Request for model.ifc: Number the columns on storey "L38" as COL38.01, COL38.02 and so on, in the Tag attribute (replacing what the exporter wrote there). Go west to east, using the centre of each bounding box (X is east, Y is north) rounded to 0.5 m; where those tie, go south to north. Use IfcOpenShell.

First a look at what the model holds.

```python
import ifcopenshell
import ifcopenshell.util.element
import ifcopenshell.util.placement

model = ifcopenshell.open("model.ifc")
print(model.schema)
storey = next(s for s in model.by_type("IfcBuildingStorey") if s.Name == "L38")
columns = [e for e in ifcopenshell.util.element.get_decomposition(storey) if e.is_a("IfcColumn")]
for e in sorted(columns, key=lambda e: e.id()):
    origin = ifcopenshell.util.placement.get_local_placement(e.ObjectPlacement)[:3, 3]
    print(e.id(), e.Tag, e.Name, origin.round(2) + 0.0, sep=" | ")
```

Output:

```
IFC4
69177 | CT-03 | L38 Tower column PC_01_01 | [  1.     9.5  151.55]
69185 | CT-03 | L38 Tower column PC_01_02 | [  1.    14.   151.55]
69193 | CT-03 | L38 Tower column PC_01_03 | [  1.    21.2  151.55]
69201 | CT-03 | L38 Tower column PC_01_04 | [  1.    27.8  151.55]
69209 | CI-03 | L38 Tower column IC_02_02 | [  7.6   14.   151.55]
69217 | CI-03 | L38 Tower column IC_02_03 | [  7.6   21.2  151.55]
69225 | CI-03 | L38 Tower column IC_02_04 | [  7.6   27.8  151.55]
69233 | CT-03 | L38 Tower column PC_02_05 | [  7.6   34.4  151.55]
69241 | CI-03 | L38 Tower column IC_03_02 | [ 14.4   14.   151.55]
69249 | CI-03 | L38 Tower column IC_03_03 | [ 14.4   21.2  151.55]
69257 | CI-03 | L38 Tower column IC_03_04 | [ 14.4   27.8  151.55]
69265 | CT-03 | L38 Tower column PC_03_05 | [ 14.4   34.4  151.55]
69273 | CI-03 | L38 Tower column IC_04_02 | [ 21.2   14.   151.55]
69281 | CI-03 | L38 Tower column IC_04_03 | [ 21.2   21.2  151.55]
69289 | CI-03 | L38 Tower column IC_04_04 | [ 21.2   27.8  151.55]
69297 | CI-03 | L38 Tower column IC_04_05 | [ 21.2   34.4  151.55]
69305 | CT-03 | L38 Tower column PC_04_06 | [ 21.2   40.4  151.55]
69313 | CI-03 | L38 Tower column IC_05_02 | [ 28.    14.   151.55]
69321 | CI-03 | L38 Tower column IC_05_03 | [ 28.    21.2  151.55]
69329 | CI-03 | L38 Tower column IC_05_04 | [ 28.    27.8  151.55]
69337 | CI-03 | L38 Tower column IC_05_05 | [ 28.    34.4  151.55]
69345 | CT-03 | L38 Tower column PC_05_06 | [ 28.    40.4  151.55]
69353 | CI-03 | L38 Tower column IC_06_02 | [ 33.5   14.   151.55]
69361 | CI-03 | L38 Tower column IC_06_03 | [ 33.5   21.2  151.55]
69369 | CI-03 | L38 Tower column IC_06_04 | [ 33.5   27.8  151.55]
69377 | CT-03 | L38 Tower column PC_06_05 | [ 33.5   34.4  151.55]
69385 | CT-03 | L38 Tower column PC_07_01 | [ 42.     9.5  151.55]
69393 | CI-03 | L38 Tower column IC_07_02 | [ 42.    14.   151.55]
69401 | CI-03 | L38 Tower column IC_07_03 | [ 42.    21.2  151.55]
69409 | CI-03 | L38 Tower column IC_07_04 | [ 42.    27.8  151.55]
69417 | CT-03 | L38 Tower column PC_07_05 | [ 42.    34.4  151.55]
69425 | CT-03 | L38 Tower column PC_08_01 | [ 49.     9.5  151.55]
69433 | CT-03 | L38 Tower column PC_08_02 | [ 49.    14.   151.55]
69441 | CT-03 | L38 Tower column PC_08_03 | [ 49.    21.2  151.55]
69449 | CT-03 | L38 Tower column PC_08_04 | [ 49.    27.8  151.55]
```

```python
import ifcopenshell
import ifcopenshell.geom
import ifcopenshell.util.element
import ifcopenshell.util.shape

model = ifcopenshell.open("model.ifc")
settings = ifcopenshell.geom.settings()
settings.set("use-world-coords", True)


def centre(element):
    shape = ifcopenshell.geom.create_shape(settings, element)
    return ifcopenshell.util.shape.get_bbox_centroid(shape.geometry)


storey = next(s for s in model.by_type("IfcBuildingStorey") if s.Name == "L38")
columns = [e for e in ifcopenshell.util.element.get_decomposition(storey) if e.is_a("IfcColumn")]

# Insertion points can sit at a corner or the storey origin, so sort by the geometry (in metres).
centres = {e: centre(e) for e in columns}
columns.sort(key=lambda e: (round(centres[e][0] / 0.5), centres[e][1]))

for i, e in enumerate(columns, start=1):
    number = f"COL38.{i:02d}"
    e.Tag = number
    print(e.id(), number)

model.write("model_rev.ifc")
```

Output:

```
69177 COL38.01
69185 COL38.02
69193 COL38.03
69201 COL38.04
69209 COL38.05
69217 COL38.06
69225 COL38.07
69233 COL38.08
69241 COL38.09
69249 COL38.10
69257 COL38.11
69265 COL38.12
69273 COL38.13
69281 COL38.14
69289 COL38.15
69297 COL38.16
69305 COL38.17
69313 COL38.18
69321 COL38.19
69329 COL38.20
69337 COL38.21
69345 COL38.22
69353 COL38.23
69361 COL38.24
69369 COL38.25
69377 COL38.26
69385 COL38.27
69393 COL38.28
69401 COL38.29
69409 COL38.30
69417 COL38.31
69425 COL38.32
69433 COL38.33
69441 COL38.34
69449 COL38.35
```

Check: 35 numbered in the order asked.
